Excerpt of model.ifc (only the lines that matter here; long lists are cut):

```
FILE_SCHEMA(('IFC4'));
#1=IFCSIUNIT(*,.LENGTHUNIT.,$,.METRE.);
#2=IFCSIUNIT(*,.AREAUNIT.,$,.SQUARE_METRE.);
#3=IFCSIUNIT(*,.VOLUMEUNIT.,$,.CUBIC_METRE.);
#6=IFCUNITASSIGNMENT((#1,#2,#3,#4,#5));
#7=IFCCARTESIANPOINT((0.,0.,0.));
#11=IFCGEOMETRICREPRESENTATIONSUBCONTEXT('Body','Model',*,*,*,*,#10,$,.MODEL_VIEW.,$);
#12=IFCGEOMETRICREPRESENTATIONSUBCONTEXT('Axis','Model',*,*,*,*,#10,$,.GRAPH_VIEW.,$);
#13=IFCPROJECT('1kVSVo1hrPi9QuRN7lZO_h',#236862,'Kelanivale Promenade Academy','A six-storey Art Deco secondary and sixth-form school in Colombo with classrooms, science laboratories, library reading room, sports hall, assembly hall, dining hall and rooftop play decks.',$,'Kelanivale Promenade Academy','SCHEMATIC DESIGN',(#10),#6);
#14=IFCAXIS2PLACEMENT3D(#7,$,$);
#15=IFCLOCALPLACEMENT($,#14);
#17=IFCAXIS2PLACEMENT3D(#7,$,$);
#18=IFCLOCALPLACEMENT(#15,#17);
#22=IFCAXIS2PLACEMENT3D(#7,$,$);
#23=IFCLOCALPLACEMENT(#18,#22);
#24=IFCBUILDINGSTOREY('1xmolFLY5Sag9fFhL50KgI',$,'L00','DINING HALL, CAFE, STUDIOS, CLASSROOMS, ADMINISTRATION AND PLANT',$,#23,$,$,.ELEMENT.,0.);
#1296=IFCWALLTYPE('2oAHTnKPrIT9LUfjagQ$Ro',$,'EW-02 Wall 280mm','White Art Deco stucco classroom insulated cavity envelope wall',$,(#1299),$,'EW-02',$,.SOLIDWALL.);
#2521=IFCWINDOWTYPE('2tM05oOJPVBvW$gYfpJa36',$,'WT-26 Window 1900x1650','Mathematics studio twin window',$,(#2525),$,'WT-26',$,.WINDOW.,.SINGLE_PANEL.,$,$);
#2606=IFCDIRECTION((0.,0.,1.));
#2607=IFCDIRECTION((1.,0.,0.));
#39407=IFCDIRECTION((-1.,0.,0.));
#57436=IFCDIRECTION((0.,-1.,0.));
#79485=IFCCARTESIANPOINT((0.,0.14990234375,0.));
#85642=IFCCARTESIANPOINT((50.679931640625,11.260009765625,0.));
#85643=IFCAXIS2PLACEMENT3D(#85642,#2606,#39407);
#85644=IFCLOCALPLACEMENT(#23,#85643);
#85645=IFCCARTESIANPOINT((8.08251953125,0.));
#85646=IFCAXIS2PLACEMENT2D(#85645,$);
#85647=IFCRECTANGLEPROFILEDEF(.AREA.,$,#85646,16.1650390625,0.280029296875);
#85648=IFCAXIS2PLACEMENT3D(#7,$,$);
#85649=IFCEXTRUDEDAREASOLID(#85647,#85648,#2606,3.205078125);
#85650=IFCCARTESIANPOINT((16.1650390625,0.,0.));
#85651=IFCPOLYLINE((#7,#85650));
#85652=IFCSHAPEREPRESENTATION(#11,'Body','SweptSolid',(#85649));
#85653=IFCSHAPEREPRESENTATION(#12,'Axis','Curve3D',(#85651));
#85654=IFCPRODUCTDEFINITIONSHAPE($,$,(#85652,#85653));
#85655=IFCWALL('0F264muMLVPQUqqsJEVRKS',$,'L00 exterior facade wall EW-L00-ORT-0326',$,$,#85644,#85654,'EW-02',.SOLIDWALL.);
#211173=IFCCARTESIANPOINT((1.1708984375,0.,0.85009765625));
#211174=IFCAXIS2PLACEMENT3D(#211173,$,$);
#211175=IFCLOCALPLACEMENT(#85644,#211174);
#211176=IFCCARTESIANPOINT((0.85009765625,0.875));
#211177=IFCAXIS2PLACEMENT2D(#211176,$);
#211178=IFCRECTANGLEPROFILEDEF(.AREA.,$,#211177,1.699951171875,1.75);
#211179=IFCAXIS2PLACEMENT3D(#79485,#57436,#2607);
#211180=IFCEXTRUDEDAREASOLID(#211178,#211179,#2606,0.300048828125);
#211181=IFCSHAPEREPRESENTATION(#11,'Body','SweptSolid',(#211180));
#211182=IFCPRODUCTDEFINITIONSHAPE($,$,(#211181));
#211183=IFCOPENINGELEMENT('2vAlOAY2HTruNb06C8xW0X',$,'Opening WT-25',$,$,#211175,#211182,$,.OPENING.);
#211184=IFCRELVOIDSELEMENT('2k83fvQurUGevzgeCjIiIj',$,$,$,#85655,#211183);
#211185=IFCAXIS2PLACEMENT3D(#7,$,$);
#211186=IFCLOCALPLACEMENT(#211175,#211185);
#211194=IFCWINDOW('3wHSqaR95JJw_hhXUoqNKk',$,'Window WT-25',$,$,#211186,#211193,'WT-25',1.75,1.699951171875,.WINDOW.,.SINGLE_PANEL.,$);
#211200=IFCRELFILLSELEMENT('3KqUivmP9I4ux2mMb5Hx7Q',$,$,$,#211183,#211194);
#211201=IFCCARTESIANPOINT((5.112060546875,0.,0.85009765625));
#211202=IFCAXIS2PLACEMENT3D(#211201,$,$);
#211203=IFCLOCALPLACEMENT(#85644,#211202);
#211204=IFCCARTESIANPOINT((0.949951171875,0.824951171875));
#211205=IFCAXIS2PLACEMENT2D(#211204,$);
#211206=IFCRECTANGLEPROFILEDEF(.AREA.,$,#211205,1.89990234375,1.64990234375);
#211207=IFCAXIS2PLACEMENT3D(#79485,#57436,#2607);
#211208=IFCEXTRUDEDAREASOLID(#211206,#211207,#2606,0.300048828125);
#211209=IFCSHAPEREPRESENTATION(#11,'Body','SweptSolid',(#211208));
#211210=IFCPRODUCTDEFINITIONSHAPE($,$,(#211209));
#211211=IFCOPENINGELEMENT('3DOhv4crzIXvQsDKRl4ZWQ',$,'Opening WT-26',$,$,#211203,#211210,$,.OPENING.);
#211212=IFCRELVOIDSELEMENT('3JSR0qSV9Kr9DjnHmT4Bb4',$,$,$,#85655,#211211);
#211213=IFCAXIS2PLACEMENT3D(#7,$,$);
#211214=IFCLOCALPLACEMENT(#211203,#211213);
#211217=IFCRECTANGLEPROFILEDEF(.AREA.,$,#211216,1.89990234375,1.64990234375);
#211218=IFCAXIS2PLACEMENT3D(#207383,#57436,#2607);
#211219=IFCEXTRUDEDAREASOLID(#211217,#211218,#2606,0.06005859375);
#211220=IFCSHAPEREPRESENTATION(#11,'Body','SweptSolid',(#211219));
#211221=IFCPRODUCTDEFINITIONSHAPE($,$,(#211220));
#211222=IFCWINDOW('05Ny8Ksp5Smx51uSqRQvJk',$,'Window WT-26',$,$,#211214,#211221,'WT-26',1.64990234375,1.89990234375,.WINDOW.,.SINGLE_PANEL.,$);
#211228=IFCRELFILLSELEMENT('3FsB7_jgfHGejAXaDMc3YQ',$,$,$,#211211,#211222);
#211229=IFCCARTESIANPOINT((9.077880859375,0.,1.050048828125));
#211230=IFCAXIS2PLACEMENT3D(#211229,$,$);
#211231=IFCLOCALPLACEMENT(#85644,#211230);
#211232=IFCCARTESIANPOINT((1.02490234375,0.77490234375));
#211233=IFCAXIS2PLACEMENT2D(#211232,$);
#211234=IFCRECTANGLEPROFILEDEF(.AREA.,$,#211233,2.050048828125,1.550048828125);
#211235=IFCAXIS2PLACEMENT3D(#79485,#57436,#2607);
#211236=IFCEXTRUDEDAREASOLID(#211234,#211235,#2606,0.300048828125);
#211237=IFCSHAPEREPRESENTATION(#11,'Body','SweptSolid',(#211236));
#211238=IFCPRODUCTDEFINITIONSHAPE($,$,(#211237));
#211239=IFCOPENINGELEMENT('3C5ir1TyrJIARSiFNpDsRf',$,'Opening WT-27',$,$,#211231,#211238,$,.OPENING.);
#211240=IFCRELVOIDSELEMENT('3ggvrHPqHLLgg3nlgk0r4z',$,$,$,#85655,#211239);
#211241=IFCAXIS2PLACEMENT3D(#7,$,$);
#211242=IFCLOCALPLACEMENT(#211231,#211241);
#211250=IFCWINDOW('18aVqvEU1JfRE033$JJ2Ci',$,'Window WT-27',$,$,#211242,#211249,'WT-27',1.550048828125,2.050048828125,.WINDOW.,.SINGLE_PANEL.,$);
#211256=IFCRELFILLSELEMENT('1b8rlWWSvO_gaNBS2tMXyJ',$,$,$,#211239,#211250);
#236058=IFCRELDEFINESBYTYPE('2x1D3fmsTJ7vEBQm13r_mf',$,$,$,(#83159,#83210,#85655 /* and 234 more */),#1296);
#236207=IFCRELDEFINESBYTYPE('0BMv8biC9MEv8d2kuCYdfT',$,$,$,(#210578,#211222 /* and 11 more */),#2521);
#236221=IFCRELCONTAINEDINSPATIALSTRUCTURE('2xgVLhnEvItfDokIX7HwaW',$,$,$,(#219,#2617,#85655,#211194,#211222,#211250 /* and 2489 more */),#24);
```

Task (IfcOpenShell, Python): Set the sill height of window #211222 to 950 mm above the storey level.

```python
import numpy as np
import ifcopenshell
import ifcopenshell.api.geometry
import ifcopenshell.geom
import ifcopenshell.util.element
import ifcopenshell.util.placement
import ifcopenshell.util.shape
import ifcopenshell.util.unit

model = ifcopenshell.open("model.ifc")
unit_scale = ifcopenshell.util.unit.calculate_unit_scale(model)

window = model.by_guid("05Ny8Ksp5Smx51uSqRQvJk")
opening = window.FillsVoids[0].RelatingOpeningElement
storey = ifcopenshell.util.element.get_container(window, ifc_class="IfcBuildingStorey")
level = ifcopenshell.util.placement.get_local_placement(storey.ObjectPlacement)[2, 3]

# The opening's origin need not be at the sill, so measure its lowest point.
shape = ifcopenshell.geom.create_shape(ifcopenshell.geom.settings(), opening)
bottom = ifcopenshell.util.shape.get_shape_bottom_elevation(shape, shape.geometry) / unit_scale
dz = level + 0.95 / unit_scale - bottom

shift = np.array([0.0, 0.0, dz])
# The window is placed relative to its opening, so it follows when the opening moves.
matrix = ifcopenshell.util.placement.get_local_placement(opening.ObjectPlacement)
matrix[:3, 3] += shift
ifcopenshell.api.geometry.edit_object_placement(
    model, product=opening, matrix=matrix, is_si=False, should_transform_children=True
)

print(f"moved by {dz * unit_scale:+.3f} m")

model.write("model_edited.ifc")
```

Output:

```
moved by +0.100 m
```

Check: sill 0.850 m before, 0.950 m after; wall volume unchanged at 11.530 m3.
